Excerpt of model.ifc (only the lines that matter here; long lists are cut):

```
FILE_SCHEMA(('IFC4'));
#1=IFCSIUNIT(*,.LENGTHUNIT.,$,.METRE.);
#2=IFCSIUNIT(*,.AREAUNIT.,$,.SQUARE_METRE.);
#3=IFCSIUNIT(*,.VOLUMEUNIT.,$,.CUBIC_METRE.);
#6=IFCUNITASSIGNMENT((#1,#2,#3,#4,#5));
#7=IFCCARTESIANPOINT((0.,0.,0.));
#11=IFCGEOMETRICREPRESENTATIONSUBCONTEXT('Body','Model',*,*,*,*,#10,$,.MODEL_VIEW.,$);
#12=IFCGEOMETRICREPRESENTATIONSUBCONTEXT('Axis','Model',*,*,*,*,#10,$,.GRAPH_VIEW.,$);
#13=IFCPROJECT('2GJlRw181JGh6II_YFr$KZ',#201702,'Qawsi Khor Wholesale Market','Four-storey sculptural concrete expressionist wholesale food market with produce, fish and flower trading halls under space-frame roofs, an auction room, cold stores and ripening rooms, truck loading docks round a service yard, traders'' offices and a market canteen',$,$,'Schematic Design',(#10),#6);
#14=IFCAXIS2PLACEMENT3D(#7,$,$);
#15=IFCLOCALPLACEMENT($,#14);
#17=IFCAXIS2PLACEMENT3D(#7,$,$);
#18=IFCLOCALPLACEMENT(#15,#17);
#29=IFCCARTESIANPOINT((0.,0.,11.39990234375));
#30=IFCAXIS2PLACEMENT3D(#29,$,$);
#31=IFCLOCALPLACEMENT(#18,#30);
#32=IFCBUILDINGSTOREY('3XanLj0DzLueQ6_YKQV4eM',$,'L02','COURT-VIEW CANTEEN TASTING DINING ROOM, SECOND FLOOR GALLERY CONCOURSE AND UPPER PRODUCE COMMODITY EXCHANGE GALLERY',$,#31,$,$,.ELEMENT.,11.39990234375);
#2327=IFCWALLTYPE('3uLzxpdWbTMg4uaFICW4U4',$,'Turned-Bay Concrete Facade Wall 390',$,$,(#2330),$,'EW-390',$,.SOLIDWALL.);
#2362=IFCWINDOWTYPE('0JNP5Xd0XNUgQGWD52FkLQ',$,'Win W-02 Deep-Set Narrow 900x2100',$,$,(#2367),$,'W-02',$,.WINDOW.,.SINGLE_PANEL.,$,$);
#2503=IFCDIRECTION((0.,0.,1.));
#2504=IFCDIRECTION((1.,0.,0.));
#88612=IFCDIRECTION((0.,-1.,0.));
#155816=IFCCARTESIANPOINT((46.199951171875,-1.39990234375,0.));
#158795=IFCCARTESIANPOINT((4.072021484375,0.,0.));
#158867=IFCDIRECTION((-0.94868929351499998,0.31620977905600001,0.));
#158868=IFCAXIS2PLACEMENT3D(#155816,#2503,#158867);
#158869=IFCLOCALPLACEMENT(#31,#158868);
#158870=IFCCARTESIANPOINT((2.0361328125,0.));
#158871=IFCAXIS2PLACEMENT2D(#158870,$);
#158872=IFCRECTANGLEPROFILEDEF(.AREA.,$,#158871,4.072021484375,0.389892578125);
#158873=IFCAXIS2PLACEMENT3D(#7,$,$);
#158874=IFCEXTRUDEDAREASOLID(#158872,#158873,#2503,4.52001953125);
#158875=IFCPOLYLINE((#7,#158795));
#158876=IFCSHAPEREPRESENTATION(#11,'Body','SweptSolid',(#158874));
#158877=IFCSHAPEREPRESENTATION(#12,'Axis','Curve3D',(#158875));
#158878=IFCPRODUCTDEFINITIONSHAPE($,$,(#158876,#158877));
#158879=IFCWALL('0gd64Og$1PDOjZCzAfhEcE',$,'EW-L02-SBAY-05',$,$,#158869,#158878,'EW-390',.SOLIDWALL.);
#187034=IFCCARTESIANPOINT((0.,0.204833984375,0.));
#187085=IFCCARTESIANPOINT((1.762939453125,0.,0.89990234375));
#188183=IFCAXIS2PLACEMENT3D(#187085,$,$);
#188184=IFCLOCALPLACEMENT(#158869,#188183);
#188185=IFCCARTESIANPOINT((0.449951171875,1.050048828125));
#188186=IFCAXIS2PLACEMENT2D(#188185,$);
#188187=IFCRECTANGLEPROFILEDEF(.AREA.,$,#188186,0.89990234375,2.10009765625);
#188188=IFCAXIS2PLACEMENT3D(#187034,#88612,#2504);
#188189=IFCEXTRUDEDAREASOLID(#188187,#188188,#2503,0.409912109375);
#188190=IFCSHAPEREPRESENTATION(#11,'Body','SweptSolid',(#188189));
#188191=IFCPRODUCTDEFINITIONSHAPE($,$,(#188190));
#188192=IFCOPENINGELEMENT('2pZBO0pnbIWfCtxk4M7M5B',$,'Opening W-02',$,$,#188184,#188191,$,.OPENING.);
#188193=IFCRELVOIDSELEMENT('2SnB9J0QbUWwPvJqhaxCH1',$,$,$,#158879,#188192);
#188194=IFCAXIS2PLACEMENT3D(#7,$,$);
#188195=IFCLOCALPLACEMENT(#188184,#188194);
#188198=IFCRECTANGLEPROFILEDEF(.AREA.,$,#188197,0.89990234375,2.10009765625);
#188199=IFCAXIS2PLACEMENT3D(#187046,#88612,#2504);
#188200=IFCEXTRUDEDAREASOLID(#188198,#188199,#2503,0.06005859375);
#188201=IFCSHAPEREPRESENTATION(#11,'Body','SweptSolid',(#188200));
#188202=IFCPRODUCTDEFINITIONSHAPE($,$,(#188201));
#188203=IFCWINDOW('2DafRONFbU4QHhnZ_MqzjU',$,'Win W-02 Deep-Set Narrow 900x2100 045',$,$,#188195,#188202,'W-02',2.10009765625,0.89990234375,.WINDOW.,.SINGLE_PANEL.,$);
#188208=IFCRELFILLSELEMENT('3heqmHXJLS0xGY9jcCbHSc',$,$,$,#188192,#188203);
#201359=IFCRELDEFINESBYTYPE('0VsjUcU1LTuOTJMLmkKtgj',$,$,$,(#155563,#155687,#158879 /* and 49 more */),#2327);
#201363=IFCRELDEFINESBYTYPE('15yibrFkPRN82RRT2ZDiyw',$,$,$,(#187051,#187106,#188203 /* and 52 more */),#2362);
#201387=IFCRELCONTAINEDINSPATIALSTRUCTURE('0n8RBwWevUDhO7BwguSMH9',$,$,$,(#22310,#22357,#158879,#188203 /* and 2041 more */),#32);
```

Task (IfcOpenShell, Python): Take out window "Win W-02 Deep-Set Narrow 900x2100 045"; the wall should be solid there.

```python
import ifcopenshell
import ifcopenshell.api.feature
import ifcopenshell.api.root
import ifcopenshell.geom
import ifcopenshell.util.shape

model = ifcopenshell.open("model.ifc")
settings = ifcopenshell.geom.settings()


def volume(element):
    """Net volume in cubic metres, openings subtracted."""
    shape = ifcopenshell.geom.create_shape(settings, element)
    return ifcopenshell.util.shape.get_volume(shape.geometry)


window = model.by_guid("2DafRONFbU4QHhnZ_MqzjU")
opening = window.FillsVoids[0].RelatingOpeningElement
wall = opening.VoidsElements[0].RelatingBuildingElement
before = volume(wall)

ifcopenshell.api.root.remove_product(model, product=window)
ifcopenshell.api.feature.remove_feature(model, feature=opening)

after = volume(wall)

print(f"wall volume {before:.3f} -> {after:.3f} m3")

model.write("model-out.ifc")
```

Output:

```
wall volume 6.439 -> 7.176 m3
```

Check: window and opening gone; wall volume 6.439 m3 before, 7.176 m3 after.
